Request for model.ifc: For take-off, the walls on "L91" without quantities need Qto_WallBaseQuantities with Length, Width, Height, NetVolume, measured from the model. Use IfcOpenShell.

First a look at what the model holds.

```python
import ifcopenshell
import ifcopenshell.util.element
import ifcopenshell.util.unit

model = ifcopenshell.open("model.ifc")
print(model.schema)
for unit_type in ("LENGTHUNIT", "AREAUNIT", "VOLUMEUNIT"):
    print(unit_type, ifcopenshell.util.unit.calculate_unit_scale(model, unit_type))
storey = next(s for s in model.by_type("IfcBuildingStorey") if s.Name == "L91")
walls = [e for e in ifcopenshell.util.element.get_decomposition(storey) if e.is_a("IfcWall")]
for e in sorted(walls, key=lambda e: e.id()):
    print(e.id(), e.is_a(), e.Name, list(ifcopenshell.util.element.get_psets(e, qtos_only=True)), sep=" | ")
```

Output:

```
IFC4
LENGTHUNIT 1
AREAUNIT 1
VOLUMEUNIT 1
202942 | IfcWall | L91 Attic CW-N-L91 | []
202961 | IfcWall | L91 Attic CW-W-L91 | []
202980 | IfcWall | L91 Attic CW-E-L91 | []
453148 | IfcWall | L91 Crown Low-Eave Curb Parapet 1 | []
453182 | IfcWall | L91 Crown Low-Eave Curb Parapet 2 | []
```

```python
import ifcopenshell
import ifcopenshell.api.pset
import ifcopenshell.geom
import ifcopenshell.util.element
import ifcopenshell.util.shape
import ifcopenshell.util.unit

model = ifcopenshell.open("model.ifc")
unit_scale = ifcopenshell.util.unit.calculate_unit_scale(model)
volume_scale = ifcopenshell.util.unit.calculate_unit_scale(model, "VOLUMEUNIT")
settings = ifcopenshell.geom.settings()

storey = next(s for s in model.by_type("IfcBuildingStorey") if s.Name == "L91")
walls = [e for e in ifcopenshell.util.element.get_decomposition(storey) if e.is_a("IfcWall")]

for e in sorted(walls, key=lambda e: e.id()):
    if ifcopenshell.util.element.get_psets(e, qtos_only=True, should_inherit=False):
        continue
    # Geometry comes back in metres, in the element's own axes.
    shape = ifcopenshell.geom.create_shape(settings, e)
    values = {
        "Length": ifcopenshell.util.shape.get_x(shape.geometry) / unit_scale,
        "Width": ifcopenshell.util.shape.get_y(shape.geometry) / unit_scale,
        "Height": ifcopenshell.util.shape.get_z(shape.geometry) / unit_scale,
        "NetVolume": ifcopenshell.util.shape.get_volume(shape.geometry) / volume_scale,
    }
    qto = ifcopenshell.api.pset.add_qto(model, product=e, name="Qto_WallBaseQuantities")
    ifcopenshell.api.pset.edit_qto(model, qto=qto, properties=values)
    print(e.id(), {k: round(v, 3) for k, v in values.items()})

model.write("model_edited.ifc")
```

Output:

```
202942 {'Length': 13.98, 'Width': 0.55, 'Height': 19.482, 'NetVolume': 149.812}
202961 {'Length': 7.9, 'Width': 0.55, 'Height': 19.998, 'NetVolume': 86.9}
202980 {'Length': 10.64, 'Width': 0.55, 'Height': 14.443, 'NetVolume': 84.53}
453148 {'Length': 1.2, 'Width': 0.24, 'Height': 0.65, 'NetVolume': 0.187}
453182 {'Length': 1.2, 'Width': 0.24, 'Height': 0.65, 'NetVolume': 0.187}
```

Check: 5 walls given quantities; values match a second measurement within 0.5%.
